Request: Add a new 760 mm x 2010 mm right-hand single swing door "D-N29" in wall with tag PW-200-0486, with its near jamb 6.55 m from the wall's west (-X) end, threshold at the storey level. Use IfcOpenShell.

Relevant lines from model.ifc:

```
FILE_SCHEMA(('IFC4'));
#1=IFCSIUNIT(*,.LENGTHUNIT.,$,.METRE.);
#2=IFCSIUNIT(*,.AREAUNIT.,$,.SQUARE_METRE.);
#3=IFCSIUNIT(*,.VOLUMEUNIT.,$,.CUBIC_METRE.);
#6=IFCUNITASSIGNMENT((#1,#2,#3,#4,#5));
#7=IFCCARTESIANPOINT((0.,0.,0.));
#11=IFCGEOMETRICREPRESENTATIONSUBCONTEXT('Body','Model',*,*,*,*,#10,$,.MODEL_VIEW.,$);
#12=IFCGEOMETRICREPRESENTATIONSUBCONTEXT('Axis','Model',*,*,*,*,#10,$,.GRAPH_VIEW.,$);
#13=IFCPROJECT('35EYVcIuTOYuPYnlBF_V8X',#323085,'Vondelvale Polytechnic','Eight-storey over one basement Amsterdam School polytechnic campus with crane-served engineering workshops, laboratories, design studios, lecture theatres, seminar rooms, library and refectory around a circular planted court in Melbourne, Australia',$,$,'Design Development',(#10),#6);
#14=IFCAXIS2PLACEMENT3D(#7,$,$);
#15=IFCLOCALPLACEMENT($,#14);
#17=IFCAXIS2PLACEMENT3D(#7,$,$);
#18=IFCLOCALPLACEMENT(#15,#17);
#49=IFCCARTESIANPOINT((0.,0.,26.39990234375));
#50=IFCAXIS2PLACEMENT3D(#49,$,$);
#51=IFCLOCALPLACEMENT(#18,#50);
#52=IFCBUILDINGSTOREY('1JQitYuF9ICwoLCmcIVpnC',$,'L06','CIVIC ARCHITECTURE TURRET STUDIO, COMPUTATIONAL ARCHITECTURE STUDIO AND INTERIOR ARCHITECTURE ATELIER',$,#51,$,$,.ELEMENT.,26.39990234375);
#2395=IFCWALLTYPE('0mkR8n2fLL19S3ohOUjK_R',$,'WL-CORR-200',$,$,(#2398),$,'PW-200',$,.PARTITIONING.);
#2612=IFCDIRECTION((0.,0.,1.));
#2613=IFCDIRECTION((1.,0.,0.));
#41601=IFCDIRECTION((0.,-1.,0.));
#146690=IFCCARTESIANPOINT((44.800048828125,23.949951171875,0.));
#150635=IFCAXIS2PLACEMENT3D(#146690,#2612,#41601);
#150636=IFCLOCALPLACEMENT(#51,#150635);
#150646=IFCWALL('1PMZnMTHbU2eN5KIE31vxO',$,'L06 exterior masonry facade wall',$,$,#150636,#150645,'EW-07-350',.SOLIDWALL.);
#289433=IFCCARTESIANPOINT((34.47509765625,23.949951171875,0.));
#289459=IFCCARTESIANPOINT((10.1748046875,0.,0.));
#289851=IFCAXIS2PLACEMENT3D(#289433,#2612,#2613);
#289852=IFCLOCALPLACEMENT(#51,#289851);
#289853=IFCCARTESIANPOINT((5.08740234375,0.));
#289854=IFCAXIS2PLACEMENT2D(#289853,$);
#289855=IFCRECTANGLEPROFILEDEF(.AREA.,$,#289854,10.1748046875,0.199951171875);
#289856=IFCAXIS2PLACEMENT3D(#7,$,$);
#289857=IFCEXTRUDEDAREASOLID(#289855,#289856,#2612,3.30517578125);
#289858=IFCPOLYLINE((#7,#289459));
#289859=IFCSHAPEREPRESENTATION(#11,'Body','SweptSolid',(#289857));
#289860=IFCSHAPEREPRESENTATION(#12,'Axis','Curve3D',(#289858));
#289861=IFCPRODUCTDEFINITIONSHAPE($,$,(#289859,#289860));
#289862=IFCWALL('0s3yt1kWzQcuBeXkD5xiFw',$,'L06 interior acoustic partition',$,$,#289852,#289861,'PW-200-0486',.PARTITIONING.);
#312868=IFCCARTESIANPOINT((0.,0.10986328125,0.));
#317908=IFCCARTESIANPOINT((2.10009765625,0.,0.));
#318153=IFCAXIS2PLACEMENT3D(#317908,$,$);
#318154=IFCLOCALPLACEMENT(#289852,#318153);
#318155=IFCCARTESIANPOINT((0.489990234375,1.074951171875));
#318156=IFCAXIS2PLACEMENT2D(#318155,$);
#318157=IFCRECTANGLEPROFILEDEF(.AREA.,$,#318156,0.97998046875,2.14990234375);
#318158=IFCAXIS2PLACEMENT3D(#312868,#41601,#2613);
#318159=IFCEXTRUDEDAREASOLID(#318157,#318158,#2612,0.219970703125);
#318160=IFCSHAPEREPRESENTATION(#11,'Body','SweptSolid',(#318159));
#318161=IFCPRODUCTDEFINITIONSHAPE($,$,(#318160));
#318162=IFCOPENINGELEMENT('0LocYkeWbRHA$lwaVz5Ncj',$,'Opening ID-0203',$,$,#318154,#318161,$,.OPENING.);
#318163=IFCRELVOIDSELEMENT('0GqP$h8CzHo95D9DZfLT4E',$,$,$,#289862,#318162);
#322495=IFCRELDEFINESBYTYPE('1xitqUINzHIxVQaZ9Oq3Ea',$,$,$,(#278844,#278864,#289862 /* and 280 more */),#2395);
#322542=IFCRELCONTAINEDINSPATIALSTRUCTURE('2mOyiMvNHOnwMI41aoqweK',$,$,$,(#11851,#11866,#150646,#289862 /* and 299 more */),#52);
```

```python
import numpy as np
import ifcopenshell
import ifcopenshell.api.feature
import ifcopenshell.api.geometry
import ifcopenshell.api.root
import ifcopenshell.api.spatial
import ifcopenshell.geom
import ifcopenshell.util.element
import ifcopenshell.util.placement
import ifcopenshell.util.representation
import ifcopenshell.util.shape
import ifcopenshell.util.unit

model = ifcopenshell.open("model.ifc")
unit_scale = ifcopenshell.util.unit.calculate_unit_scale(model)
settings = ifcopenshell.geom.settings()


def volume(element):
    """Net volume in cubic metres, openings subtracted."""
    shape = ifcopenshell.geom.create_shape(settings, element)
    return ifcopenshell.util.shape.get_volume(shape.geometry)


wall = model.by_id(289862)
storey = ifcopenshell.util.element.get_container(wall, ifc_class="IfcBuildingStorey")
context = ifcopenshell.util.representation.get_context(model, "Model", "Body", "MODEL_VIEW")
before = volume(wall)

width, height, from_end, sill = 0.76, 2.01, 6.55, 0.0  # metres

# The wall runs along its own X axis, and the end named is its -X end.
wall_shape = ifcopenshell.geom.create_shape(settings, wall)
x, y, z = ifcopenshell.util.shape.get_vertices(wall_shape.geometry).T
start = x.min() + from_end
face, thickness = float(y.min()), float(y.max() - y.min())
wall_matrix = ifcopenshell.util.placement.get_local_placement(wall.ObjectPlacement)
level = ifcopenshell.util.placement.get_local_placement(storey.ObjectPlacement)[2, 3]


def in_wall(x, y):
    """Placement at x, y metres in the wall's axes, at sill height."""
    matrix = wall_matrix.copy()
    matrix[:, 3] = wall_matrix @ np.array([x / unit_scale, y / unit_scale, 0.0, 1.0])
    matrix[2, 3] = level + sill / unit_scale
    return matrix


# Opening: a box that overshoots both wall faces by 50 mm.
opening = ifcopenshell.api.root.create_entity(model, ifc_class="IfcOpeningElement", predefined_type="OPENING")
box = ifcopenshell.api.geometry.add_wall_representation(
    model, context=context, length=width, height=height, thickness=thickness + 0.1
)
ifcopenshell.api.geometry.assign_representation(model, product=opening, representation=box)
ifcopenshell.api.geometry.edit_object_placement(model, product=opening, matrix=in_wall(start, face - 0.05), is_si=False)
ifcopenshell.api.feature.add_feature(model, feature=opening, element=wall)

door = ifcopenshell.api.root.create_entity(model, ifc_class="IfcDoor", name="D-N29", predefined_type="DOOR")
door.OverallWidth, door.OverallHeight = width / unit_scale, height / unit_scale
door.OperationType = "SINGLE_SWING_RIGHT"
body = ifcopenshell.api.geometry.add_door_representation(
    model,
    context=context,
    overall_width=door.OverallWidth,
    overall_height=door.OverallHeight,
    operation_type="SINGLE_SWING_RIGHT",
    lining_properties={"LiningDepth": thickness / unit_scale, "ThresholdDepth": thickness / unit_scale},
)
ifcopenshell.api.geometry.assign_representation(model, product=door, representation=body)
ifcopenshell.api.spatial.assign_container(model, products=[door], relating_structure=storey)
ifcopenshell.api.feature.add_filling(model, opening=opening, element=door)

# The lining spans the wall, so the door starts at the wall face.
ifcopenshell.api.geometry.edit_object_placement(model, product=door, matrix=in_wall(start, face), is_si=False)

after = volume(wall)

print(f"wall volume {before:.3f} -> {after:.3f} m3")

model.write("model_rev.ifc")
```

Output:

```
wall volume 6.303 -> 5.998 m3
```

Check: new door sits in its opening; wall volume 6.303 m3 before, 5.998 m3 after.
